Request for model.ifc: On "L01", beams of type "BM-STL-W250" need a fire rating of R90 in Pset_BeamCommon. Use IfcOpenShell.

First a look at what the model holds.

```python
import ifcopenshell
import ifcopenshell.util.element

model = ifcopenshell.open("model.ifc")
print(model.schema)
storey = next(s for s in model.by_type("IfcBuildingStorey") if s.Name == "L01")
beams = [e for e in ifcopenshell.util.element.get_decomposition(storey) if e.is_a("IfcBeam")]
seen = {}
for e in beams:
    element_type = ifcopenshell.util.element.get_type(e)
    key = (element_type.Name if element_type != e and element_type else None, ifcopenshell.util.element.get_pset(e, "Pset_BeamCommon", "FireRating"))
    seen[key] = seen.get(key, 0) + 1
for (name, value), count in sorted(seen.items(), key=str):
    print(count, "x", name, "|", value)
```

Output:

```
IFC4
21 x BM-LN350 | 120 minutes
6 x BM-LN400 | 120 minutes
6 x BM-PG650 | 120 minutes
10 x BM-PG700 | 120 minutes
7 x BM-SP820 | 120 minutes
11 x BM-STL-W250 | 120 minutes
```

```python
import ifcopenshell
import ifcopenshell.api.pset
import ifcopenshell.util.element

model = ifcopenshell.open("model.ifc")

storey = next(s for s in model.by_type("IfcBuildingStorey") if s.Name == "L01")
beams = [e for e in ifcopenshell.util.element.get_decomposition(storey) if e.is_a("IfcBeam")]

count = 0
for e in beams:
    element_type = ifcopenshell.util.element.get_type(e)
    if element_type in (None, e) or element_type.Name != "BM-STL-W250":
        continue
    # add_pset returns the element's existing set when there is one.
    pset = ifcopenshell.api.pset.add_pset(model, product=e, name="Pset_BeamCommon")
    ifcopenshell.api.pset.edit_pset(model, pset=pset, properties={"FireRating": "R90"})
    count += 1

print(count, "beams updated")

model.write("model_rev.ifc")
```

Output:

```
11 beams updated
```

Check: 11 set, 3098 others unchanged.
